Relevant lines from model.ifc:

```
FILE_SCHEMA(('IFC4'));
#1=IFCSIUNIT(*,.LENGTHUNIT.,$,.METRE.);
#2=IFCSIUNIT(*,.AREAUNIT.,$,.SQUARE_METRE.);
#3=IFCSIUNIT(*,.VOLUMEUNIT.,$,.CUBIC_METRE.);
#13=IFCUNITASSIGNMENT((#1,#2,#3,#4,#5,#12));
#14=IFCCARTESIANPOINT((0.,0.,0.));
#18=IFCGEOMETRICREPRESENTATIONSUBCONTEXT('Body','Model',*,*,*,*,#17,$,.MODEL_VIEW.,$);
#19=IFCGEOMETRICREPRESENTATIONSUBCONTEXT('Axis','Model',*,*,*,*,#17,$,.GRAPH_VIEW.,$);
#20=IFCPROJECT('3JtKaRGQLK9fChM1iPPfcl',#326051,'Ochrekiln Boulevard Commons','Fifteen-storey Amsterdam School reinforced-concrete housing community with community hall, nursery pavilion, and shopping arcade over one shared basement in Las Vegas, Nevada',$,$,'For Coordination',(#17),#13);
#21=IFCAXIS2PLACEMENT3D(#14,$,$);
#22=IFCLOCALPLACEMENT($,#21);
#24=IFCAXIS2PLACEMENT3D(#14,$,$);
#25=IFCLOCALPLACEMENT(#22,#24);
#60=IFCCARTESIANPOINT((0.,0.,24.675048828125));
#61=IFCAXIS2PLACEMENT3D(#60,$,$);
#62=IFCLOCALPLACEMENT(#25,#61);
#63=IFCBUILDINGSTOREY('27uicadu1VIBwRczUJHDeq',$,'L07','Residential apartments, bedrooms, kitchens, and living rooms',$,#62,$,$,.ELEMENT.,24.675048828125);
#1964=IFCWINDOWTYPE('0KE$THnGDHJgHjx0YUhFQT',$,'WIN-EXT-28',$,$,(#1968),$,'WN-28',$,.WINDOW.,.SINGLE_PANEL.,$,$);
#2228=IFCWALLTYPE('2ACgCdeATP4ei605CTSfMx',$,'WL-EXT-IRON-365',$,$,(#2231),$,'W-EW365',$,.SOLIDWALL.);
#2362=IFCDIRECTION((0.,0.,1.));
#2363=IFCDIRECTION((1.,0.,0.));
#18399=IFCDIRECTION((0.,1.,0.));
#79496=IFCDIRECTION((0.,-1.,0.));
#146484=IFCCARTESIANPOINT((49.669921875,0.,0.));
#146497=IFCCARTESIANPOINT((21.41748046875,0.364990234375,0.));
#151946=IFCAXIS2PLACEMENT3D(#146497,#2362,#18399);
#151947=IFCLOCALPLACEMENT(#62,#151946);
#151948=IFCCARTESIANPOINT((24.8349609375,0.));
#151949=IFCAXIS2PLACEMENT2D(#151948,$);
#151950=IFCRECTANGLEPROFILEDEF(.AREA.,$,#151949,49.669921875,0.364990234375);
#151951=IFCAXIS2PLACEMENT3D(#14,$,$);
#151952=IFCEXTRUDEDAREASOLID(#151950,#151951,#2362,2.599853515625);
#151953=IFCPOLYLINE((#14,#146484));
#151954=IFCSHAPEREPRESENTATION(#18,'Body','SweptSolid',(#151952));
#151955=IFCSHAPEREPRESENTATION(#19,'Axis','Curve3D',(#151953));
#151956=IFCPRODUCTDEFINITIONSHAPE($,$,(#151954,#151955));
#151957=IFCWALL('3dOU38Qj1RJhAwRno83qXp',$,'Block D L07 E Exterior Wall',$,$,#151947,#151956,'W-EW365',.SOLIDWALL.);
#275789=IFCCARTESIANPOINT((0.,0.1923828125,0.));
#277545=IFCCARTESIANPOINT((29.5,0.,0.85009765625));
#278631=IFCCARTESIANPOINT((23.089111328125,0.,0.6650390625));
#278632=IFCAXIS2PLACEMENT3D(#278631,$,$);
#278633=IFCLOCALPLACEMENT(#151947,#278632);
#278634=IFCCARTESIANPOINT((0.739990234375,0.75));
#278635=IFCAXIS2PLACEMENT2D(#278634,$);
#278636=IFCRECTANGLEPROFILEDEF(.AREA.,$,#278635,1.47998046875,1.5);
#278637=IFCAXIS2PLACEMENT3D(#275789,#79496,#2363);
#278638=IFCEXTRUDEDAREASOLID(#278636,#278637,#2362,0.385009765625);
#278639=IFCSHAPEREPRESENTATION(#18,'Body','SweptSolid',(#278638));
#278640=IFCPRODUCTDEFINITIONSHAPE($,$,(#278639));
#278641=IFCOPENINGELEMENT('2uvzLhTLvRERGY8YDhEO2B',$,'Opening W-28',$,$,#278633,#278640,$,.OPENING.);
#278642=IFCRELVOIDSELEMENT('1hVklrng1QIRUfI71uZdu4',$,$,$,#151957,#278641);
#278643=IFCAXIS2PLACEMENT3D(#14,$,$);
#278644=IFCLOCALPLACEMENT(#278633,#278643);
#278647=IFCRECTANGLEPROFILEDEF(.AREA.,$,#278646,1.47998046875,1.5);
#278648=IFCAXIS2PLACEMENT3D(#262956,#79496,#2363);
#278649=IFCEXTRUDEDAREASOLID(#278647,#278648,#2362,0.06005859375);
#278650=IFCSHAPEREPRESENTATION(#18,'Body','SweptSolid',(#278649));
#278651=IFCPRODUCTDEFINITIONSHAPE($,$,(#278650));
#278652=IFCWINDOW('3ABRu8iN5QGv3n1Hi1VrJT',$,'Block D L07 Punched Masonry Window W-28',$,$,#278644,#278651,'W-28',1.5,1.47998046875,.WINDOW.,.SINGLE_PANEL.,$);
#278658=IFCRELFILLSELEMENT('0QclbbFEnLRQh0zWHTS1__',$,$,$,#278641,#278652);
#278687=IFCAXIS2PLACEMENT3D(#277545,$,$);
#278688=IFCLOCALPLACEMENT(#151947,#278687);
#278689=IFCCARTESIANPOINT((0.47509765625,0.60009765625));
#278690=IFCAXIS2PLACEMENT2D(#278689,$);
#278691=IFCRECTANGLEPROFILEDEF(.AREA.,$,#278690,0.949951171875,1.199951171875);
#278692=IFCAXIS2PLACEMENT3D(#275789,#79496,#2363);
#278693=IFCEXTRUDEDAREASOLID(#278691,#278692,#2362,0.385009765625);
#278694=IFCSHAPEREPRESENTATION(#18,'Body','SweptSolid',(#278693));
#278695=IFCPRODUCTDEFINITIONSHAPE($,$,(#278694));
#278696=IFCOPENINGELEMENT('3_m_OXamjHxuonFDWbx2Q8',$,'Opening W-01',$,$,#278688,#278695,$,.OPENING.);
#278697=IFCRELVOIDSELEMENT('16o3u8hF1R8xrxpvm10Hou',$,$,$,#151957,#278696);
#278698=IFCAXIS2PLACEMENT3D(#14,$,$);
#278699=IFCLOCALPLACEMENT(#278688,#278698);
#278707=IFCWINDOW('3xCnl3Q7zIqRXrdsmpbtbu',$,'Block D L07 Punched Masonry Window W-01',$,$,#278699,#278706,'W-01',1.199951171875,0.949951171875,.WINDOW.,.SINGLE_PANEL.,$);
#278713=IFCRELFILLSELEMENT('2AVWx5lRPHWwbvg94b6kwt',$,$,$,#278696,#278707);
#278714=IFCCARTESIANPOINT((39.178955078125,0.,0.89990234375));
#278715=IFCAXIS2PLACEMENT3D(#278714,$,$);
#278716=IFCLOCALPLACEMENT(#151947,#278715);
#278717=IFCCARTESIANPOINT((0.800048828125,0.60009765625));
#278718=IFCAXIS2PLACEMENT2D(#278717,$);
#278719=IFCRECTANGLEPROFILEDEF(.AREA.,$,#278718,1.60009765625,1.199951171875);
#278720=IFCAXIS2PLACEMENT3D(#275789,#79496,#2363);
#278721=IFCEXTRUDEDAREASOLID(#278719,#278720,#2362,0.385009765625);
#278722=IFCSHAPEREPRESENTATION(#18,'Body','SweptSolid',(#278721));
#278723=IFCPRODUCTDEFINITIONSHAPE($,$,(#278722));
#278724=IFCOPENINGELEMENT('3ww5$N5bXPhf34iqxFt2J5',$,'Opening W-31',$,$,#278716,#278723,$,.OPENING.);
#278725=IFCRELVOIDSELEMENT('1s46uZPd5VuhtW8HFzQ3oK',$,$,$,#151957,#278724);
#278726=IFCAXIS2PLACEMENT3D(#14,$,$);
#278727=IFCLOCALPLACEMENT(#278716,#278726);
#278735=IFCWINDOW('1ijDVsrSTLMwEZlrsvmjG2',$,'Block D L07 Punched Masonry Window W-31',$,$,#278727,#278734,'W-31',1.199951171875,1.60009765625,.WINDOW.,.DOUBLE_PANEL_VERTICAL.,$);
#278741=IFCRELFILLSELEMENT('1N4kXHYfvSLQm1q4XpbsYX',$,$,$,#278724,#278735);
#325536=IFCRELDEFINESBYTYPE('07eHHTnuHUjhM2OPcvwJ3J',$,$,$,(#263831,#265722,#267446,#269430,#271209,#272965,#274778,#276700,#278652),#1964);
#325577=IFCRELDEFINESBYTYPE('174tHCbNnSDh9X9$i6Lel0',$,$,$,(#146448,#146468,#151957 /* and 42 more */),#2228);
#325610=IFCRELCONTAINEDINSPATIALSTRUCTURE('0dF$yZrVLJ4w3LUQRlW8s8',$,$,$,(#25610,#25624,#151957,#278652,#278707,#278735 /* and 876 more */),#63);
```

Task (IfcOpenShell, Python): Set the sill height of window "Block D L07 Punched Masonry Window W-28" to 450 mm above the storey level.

```python
import numpy as np
import ifcopenshell
import ifcopenshell.api.geometry
import ifcopenshell.geom
import ifcopenshell.util.element
import ifcopenshell.util.placement
import ifcopenshell.util.shape
import ifcopenshell.util.unit

model = ifcopenshell.open("model.ifc")
unit_scale = ifcopenshell.util.unit.calculate_unit_scale(model)

window = model.by_guid("3ABRu8iN5QGv3n1Hi1VrJT")
opening = window.FillsVoids[0].RelatingOpeningElement
storey = ifcopenshell.util.element.get_container(window, ifc_class="IfcBuildingStorey")
level = ifcopenshell.util.placement.get_local_placement(storey.ObjectPlacement)[2, 3]

# The opening's origin need not be at the sill, so measure its lowest point.
shape = ifcopenshell.geom.create_shape(ifcopenshell.geom.settings(), opening)
bottom = ifcopenshell.util.shape.get_shape_bottom_elevation(shape, shape.geometry) / unit_scale
dz = level + 0.45 - bottom

shift = np.array([0.0, 0.0, dz])
# The window is placed relative to its opening, so it follows when the opening moves.
matrix = ifcopenshell.util.placement.get_local_placement(opening.ObjectPlacement)
matrix[:3, 3] += shift
ifcopenshell.api.geometry.edit_object_placement(
    model, product=opening, matrix=matrix, is_si=False, should_transform_children=True
)

print(f"moved by {dz * unit_scale:+.3f} m")

model.write("model_rev.ifc")
```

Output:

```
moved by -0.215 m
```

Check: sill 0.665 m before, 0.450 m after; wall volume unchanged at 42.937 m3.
